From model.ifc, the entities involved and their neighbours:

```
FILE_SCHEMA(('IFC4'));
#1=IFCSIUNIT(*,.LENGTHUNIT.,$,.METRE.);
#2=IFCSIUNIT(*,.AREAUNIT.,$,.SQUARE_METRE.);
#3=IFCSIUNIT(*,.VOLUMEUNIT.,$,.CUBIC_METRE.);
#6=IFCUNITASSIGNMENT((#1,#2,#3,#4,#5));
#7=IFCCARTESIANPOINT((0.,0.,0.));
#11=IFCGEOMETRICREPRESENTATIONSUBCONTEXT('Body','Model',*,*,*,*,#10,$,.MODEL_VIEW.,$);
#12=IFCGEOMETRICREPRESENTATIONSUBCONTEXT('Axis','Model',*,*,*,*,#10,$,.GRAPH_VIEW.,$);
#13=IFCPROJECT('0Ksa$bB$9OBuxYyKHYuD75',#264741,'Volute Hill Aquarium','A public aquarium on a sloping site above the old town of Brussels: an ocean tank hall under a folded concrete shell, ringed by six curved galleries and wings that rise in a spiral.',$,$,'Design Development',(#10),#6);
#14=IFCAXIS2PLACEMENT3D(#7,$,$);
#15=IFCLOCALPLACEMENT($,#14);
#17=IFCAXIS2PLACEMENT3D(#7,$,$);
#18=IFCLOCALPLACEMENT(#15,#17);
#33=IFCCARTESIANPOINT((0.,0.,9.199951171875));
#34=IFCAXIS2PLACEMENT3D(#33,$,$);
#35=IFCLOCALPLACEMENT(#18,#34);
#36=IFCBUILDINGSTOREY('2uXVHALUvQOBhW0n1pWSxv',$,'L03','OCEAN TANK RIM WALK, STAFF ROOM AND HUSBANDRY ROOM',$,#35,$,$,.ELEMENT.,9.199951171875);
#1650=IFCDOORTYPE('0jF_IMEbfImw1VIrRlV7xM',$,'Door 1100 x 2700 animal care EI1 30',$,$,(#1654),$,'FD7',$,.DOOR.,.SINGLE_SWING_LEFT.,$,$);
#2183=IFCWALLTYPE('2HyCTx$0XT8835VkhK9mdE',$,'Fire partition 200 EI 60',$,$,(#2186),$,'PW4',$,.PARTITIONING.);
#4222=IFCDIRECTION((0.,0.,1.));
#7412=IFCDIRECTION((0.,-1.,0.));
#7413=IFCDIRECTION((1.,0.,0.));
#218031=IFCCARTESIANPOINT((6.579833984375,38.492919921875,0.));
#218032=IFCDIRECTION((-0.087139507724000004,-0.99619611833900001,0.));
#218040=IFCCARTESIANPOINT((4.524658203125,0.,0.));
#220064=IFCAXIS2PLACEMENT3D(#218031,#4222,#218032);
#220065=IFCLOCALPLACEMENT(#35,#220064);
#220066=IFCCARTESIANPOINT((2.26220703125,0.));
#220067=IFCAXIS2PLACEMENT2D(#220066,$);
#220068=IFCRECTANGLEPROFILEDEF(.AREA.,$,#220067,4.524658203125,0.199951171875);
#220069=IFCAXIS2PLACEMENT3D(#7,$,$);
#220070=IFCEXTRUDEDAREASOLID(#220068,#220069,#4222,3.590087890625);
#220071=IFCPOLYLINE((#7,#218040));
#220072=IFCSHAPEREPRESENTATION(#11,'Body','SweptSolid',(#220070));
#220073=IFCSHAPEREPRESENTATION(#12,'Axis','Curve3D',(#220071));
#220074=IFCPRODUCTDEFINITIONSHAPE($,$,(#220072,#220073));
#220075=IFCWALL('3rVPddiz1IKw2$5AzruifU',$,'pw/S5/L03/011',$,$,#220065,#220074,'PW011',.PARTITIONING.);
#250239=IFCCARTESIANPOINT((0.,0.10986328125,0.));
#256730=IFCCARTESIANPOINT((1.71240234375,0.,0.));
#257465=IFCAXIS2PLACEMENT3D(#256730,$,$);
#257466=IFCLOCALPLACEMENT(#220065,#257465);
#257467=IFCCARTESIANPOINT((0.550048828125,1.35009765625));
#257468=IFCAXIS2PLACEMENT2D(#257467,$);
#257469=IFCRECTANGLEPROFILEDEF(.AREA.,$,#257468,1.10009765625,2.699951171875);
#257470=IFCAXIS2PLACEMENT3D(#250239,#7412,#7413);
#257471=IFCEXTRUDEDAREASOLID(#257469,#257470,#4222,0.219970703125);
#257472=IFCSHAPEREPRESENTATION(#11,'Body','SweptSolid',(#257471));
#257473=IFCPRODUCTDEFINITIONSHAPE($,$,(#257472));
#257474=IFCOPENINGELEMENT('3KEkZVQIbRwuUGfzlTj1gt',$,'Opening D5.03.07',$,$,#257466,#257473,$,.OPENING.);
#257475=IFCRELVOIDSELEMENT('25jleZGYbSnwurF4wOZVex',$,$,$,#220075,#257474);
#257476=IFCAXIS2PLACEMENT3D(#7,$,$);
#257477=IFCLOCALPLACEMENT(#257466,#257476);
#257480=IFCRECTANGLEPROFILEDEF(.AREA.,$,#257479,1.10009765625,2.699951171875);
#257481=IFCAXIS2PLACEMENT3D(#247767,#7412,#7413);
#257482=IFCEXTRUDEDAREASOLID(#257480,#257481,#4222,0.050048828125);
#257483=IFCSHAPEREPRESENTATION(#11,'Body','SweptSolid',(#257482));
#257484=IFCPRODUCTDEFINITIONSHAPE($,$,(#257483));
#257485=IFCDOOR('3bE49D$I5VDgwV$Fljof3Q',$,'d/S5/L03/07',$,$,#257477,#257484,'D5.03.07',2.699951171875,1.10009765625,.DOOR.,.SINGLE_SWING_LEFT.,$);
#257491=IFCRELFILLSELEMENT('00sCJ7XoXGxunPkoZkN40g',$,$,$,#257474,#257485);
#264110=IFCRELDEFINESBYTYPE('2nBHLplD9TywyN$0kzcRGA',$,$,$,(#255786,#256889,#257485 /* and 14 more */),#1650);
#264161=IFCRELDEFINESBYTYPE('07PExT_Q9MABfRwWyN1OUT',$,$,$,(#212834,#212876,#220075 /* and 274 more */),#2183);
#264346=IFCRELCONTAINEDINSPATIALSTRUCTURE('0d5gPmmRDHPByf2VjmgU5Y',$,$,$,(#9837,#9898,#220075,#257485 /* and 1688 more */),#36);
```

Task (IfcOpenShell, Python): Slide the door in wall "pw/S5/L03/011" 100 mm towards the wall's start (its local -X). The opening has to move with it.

```python
import ifcopenshell
import ifcopenshell.api.geometry
import ifcopenshell.util.placement
import ifcopenshell.util.unit

model = ifcopenshell.open("model.ifc")
unit_scale = ifcopenshell.util.unit.calculate_unit_scale(model)

door = model.by_guid("3bE49D$I5VDgwV$Fljof3Q")
opening = door.FillsVoids[0].RelatingOpeningElement
wall = opening.VoidsElements[0].RelatingBuildingElement

wall_matrix = ifcopenshell.util.placement.get_local_placement(wall.ObjectPlacement)
shift = wall_matrix[:3, 0] * -0.1 / unit_scale
before = ifcopenshell.util.placement.get_local_placement(door.ObjectPlacement)[:3, 3].copy()

# The door is placed relative to its opening, so it follows when the opening moves.
matrix = ifcopenshell.util.placement.get_local_placement(opening.ObjectPlacement)
matrix[:3, 3] += shift
ifcopenshell.api.geometry.edit_object_placement(
    model, product=opening, matrix=matrix, is_si=False, should_transform_children=True
)

after = ifcopenshell.util.placement.get_local_placement(door.ObjectPlacement)[:3, 3]
print("door moved by", (after - before).round(3) + 0.0)

model.write("model_rev.ifc")
```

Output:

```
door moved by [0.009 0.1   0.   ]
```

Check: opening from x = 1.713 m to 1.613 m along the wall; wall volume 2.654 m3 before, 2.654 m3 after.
